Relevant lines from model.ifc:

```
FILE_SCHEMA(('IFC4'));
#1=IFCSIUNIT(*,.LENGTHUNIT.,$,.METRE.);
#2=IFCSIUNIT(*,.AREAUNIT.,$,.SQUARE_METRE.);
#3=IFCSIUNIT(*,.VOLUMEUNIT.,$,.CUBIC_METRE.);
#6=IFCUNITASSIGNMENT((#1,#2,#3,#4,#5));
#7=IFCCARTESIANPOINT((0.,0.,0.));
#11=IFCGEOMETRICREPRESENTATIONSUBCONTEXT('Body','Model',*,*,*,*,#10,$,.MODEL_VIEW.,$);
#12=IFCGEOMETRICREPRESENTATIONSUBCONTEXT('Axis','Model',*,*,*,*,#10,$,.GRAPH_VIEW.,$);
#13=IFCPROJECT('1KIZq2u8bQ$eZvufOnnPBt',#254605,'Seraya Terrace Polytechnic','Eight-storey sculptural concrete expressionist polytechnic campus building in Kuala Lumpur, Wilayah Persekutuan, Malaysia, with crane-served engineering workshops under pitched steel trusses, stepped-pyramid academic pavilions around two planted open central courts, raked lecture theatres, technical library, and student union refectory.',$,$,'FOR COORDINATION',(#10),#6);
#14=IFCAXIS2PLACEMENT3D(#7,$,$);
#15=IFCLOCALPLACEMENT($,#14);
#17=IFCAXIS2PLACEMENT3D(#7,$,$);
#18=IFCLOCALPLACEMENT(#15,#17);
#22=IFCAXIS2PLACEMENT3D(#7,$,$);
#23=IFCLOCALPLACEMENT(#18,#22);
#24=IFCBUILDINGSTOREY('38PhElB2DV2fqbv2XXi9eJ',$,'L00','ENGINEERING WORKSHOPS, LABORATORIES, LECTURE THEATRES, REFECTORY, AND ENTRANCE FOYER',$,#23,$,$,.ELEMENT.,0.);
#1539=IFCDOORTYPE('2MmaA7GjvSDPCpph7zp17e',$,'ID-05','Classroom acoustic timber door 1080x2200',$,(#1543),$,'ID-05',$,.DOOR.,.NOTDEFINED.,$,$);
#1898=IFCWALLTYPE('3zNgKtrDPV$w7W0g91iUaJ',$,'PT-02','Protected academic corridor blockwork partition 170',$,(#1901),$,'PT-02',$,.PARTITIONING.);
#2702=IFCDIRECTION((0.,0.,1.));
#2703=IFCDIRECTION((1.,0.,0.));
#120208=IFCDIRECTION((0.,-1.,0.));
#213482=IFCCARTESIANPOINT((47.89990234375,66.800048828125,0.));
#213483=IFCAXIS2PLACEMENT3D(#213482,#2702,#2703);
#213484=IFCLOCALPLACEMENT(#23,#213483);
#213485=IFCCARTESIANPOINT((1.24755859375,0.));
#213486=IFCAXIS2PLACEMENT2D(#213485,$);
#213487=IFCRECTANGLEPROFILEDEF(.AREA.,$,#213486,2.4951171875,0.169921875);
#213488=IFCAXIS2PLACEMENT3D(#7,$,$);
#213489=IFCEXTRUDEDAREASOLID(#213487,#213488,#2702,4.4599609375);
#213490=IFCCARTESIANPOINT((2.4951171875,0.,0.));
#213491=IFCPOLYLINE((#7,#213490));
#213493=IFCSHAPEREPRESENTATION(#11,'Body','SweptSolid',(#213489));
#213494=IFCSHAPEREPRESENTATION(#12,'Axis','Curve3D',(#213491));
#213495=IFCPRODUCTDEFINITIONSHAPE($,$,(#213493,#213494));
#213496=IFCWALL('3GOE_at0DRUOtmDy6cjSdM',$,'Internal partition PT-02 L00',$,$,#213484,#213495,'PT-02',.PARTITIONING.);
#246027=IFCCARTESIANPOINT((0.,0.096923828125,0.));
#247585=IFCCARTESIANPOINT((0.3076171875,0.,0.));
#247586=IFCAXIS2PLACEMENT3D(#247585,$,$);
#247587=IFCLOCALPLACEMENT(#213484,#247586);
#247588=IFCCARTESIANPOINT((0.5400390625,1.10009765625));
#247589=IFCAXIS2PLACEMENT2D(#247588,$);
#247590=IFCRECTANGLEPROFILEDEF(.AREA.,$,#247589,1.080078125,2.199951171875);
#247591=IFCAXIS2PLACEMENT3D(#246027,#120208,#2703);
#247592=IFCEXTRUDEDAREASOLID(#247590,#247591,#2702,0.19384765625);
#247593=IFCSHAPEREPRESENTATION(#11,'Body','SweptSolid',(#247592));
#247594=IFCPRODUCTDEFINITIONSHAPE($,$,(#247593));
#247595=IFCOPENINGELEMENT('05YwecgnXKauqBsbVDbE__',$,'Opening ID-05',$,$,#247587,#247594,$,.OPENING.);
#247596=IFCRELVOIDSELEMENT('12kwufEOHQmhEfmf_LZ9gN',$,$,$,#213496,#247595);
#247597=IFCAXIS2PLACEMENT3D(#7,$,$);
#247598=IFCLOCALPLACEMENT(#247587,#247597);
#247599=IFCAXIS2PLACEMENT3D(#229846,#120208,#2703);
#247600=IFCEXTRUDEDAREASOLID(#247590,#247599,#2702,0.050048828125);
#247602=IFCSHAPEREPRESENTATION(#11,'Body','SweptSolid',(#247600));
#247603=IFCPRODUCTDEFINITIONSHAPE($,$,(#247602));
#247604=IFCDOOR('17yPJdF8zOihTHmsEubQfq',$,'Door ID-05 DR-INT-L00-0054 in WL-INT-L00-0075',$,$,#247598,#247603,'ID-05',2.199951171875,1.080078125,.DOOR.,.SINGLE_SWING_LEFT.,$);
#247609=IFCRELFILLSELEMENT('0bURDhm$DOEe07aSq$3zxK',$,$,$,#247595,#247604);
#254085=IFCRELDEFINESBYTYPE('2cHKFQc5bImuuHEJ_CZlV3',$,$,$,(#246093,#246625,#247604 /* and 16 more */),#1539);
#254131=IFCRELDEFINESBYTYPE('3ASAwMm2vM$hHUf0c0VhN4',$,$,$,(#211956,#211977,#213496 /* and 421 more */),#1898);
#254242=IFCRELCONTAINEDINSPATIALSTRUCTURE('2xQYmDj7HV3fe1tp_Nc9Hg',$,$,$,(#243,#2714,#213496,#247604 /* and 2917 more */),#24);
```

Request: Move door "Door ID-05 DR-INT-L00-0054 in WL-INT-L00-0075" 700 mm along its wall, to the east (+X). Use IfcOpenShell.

```python
import ifcopenshell
import ifcopenshell.api.geometry
import ifcopenshell.util.placement

model = ifcopenshell.open("model.ifc")

door = model.by_guid("17yPJdF8zOihTHmsEubQfq")
opening = door.FillsVoids[0].RelatingOpeningElement
wall = opening.VoidsElements[0].RelatingBuildingElement

wall_matrix = ifcopenshell.util.placement.get_local_placement(wall.ObjectPlacement)
shift = wall_matrix[:3, 0] * 0.7
before = ifcopenshell.util.placement.get_local_placement(door.ObjectPlacement)[:3, 3].copy()

# The door is placed relative to its opening, so it follows when the opening moves.
matrix = ifcopenshell.util.placement.get_local_placement(opening.ObjectPlacement)
matrix[:3, 3] += shift
ifcopenshell.api.geometry.edit_object_placement(
    model, product=opening, matrix=matrix, is_si=False, should_transform_children=True
)

after = ifcopenshell.util.placement.get_local_placement(door.ObjectPlacement)[:3, 3]
print("door moved by", (after - before).round(3) + 0.0)

model.write("model_v2.ifc")
```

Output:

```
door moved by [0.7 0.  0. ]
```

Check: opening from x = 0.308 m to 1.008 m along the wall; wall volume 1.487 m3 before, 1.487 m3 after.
